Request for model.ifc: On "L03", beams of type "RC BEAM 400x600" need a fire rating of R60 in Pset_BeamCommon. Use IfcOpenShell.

First a look at what the model holds.

```python
import ifcopenshell
import ifcopenshell.util.element

model = ifcopenshell.open("model.ifc")
print(model.schema)
storey = next(s for s in model.by_type("IfcBuildingStorey") if s.Name == "L03")
beams = [e for e in ifcopenshell.util.element.get_decomposition(storey) if e.is_a("IfcBeam")]
seen = {}
for e in beams:
    element_type = ifcopenshell.util.element.get_type(e)
    key = (element_type.Name if element_type != e and element_type else None, ifcopenshell.util.element.get_pset(e, "Pset_BeamCommon", "FireRating"))
    seen[key] = seen.get(key, 0) + 1
for (name, value), count in sorted(seen.items(), key=str):
    print(count, "x", name, "|", value)
```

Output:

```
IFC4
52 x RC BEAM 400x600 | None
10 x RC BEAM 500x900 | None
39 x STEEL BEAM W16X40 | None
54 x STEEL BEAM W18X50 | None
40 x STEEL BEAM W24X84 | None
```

```python
import ifcopenshell
import ifcopenshell.api.pset
import ifcopenshell.util.element

model = ifcopenshell.open("model.ifc")

storey = next(s for s in model.by_type("IfcBuildingStorey") if s.Name == "L03")
beams = [e for e in ifcopenshell.util.element.get_decomposition(storey) if e.is_a("IfcBeam")]

count = 0
for e in beams:
    element_type = ifcopenshell.util.element.get_type(e)
    if element_type in (None, e) or element_type.Name != "RC BEAM 400x600":
        continue
    # add_pset returns the element's existing set when there is one.
    pset = ifcopenshell.api.pset.add_pset(model, product=e, name="Pset_BeamCommon")
    ifcopenshell.api.pset.edit_pset(model, pset=pset, properties={"FireRating": "R60"})
    count += 1

print(count, "beams updated")

model.write("model_v2.ifc")
```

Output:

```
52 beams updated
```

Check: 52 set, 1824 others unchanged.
